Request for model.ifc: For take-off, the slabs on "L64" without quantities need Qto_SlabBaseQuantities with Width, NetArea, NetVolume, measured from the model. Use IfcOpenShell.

First a look at what the model holds.

```python
import ifcopenshell
import ifcopenshell.util.element
import ifcopenshell.util.unit

model = ifcopenshell.open("model.ifc")
print(model.schema)
for unit_type in ("LENGTHUNIT", "AREAUNIT", "VOLUMEUNIT"):
    print(unit_type, ifcopenshell.util.unit.calculate_unit_scale(model, unit_type))
storey = next(s for s in model.by_type("IfcBuildingStorey") if s.Name == "L64")
slabs = [e for e in ifcopenshell.util.element.get_decomposition(storey) if e.is_a("IfcSlab")]
for e in sorted(slabs, key=lambda e: e.id()):
    print(e.id(), e.is_a(), e.Name, list(ifcopenshell.util.element.get_psets(e, qtos_only=True)), sep=" | ")
```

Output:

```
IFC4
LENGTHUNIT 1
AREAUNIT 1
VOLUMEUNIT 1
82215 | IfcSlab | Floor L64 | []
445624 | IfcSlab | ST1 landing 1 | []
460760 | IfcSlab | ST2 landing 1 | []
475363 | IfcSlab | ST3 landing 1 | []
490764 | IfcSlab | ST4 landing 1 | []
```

```python
import ifcopenshell
import ifcopenshell.api.pset
import ifcopenshell.geom
import ifcopenshell.util.element
import ifcopenshell.util.shape
import ifcopenshell.util.unit

model = ifcopenshell.open("model.ifc")
unit_scale = ifcopenshell.util.unit.calculate_unit_scale(model)
area_scale = ifcopenshell.util.unit.calculate_unit_scale(model, "AREAUNIT")
volume_scale = ifcopenshell.util.unit.calculate_unit_scale(model, "VOLUMEUNIT")
settings = ifcopenshell.geom.settings()

storey = next(s for s in model.by_type("IfcBuildingStorey") if s.Name == "L64")
slabs = [e for e in ifcopenshell.util.element.get_decomposition(storey) if e.is_a("IfcSlab")]

for e in sorted(slabs, key=lambda e: e.id()):
    if ifcopenshell.util.element.get_psets(e, qtos_only=True, should_inherit=False):
        continue
    # Geometry comes back in metres, in the element's own axes.
    shape = ifcopenshell.geom.create_shape(settings, e)
    values = {
        "Width": ifcopenshell.util.shape.get_z(shape.geometry) / unit_scale,
        "NetArea": ifcopenshell.util.shape.get_footprint_area(shape.geometry) / area_scale,
        "NetVolume": ifcopenshell.util.shape.get_volume(shape.geometry) / volume_scale,
    }
    qto = ifcopenshell.api.pset.add_qto(model, product=e, name="Qto_SlabBaseQuantities")
    ifcopenshell.api.pset.edit_qto(model, qto=qto, properties=values)
    print(e.id(), {k: round(v, 3) for k, v in values.items()})

model.write("model_rev.ifc")
```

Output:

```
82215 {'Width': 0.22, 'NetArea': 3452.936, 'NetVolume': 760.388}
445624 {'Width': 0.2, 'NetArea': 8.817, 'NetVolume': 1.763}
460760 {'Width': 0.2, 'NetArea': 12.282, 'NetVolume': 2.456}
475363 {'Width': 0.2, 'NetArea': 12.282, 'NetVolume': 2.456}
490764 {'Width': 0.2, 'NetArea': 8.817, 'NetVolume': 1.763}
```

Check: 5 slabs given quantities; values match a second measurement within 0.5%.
